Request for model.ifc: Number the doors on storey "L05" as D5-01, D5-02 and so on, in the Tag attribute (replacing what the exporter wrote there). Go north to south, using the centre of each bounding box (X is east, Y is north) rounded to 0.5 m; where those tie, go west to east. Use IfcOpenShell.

First a look at what the model holds.

```python
import ifcopenshell
import ifcopenshell.util.element
import ifcopenshell.util.placement

model = ifcopenshell.open("model.ifc")
print(model.schema)
storey = next(s for s in model.by_type("IfcBuildingStorey") if s.Name == "L05")
doors = [e for e in ifcopenshell.util.element.get_decomposition(storey) if e.is_a("IfcDoor")]
for e in sorted(doors, key=lambda e: e.id()):
    origin = ifcopenshell.util.placement.get_local_placement(e.ObjectPlacement)[:3, 3]
    print(e.id(), e.Tag, e.Name, origin.round(2) + 0.0, sep=" | ")
```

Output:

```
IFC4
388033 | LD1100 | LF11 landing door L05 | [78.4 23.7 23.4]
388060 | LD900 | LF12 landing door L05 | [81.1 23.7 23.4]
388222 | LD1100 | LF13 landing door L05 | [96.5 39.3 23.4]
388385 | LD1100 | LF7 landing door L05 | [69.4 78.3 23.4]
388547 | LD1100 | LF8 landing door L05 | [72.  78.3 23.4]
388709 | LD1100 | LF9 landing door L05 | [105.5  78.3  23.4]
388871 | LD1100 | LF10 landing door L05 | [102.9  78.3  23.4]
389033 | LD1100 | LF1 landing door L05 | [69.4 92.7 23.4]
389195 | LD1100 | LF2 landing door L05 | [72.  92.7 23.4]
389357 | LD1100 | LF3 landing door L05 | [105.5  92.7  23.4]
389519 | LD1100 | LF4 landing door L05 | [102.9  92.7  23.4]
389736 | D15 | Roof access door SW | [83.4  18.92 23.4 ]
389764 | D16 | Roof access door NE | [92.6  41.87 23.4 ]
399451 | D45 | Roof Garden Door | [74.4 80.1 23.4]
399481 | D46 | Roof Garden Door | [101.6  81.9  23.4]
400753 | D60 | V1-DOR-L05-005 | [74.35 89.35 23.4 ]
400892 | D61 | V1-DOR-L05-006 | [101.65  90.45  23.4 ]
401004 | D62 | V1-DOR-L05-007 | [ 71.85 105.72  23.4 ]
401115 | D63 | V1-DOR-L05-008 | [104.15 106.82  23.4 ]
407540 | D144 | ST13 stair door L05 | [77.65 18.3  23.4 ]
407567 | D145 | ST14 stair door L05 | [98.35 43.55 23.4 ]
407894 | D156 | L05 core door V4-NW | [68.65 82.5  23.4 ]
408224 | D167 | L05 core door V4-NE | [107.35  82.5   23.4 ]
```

```python
import ifcopenshell
import ifcopenshell.geom
import ifcopenshell.util.element
import ifcopenshell.util.shape

model = ifcopenshell.open("model.ifc")
settings = ifcopenshell.geom.settings()
settings.set("use-world-coords", True)


def centre(element):
    shape = ifcopenshell.geom.create_shape(settings, element)
    return ifcopenshell.util.shape.get_bbox_centroid(shape.geometry)


storey = next(s for s in model.by_type("IfcBuildingStorey") if s.Name == "L05")
doors = [e for e in ifcopenshell.util.element.get_decomposition(storey) if e.is_a("IfcDoor")]

# Insertion points can sit at a corner or the storey origin, so sort by the geometry (in metres).
centres = {e: centre(e) for e in doors}
doors.sort(key=lambda e: (-round(centres[e][1] / 0.5), centres[e][0]))

for i, e in enumerate(doors, start=1):
    number = f"D5-{i:02d}"
    e.Tag = number
    print(e.id(), number)

model.write("model-out.ifc")
```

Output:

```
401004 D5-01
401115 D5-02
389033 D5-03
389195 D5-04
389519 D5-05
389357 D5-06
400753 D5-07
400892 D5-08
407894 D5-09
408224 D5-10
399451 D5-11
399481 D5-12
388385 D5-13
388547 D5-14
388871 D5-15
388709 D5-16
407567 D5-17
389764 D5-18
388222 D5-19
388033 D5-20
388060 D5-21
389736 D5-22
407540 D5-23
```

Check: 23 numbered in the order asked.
